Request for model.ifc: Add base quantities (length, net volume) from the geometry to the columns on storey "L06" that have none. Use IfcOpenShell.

First a look at what the model holds.

```python
import ifcopenshell
import ifcopenshell.util.element
import ifcopenshell.util.unit

model = ifcopenshell.open("model.ifc")
print(model.schema)
for unit_type in ("LENGTHUNIT", "AREAUNIT", "VOLUMEUNIT"):
    print(unit_type, ifcopenshell.util.unit.calculate_unit_scale(model, unit_type))
storey = next(s for s in model.by_type("IfcBuildingStorey") if s.Name == "L06")
columns = [e for e in ifcopenshell.util.element.get_decomposition(storey) if e.is_a("IfcColumn")]
for e in sorted(columns, key=lambda e: e.id()):
    print(e.id(), e.is_a(), e.Name, list(ifcopenshell.util.element.get_psets(e, qtos_only=True)), sep=" | ")
```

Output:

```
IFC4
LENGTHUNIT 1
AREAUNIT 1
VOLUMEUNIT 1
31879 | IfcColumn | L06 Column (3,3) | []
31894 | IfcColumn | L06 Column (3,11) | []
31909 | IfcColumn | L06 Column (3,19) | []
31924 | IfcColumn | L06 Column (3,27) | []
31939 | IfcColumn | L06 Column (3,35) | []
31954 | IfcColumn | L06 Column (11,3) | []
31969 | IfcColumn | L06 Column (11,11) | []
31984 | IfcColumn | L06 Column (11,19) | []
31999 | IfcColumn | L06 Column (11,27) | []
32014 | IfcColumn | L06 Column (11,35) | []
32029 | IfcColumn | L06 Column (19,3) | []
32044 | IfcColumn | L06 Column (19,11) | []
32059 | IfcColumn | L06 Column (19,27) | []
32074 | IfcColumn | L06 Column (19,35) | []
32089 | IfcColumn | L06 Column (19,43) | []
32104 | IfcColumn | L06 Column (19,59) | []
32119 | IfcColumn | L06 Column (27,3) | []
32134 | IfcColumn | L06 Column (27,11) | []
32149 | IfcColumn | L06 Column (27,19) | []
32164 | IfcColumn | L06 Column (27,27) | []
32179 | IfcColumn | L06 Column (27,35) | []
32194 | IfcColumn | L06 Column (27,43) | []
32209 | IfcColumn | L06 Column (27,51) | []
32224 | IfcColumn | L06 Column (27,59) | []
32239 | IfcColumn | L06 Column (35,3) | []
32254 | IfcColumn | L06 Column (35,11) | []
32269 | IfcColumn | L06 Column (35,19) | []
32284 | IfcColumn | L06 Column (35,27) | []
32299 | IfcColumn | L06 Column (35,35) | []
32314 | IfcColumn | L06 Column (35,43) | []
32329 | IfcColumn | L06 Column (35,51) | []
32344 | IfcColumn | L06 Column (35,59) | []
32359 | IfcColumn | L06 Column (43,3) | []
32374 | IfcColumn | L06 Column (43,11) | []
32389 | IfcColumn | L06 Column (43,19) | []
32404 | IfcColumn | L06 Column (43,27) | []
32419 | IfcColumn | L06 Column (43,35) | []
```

```python
import ifcopenshell
import ifcopenshell.api.pset
import ifcopenshell.geom
import ifcopenshell.util.element
import ifcopenshell.util.shape
import ifcopenshell.util.unit

model = ifcopenshell.open("model.ifc")
unit_scale = ifcopenshell.util.unit.calculate_unit_scale(model)
volume_scale = ifcopenshell.util.unit.calculate_unit_scale(model, "VOLUMEUNIT")
settings = ifcopenshell.geom.settings()

storey = next(s for s in model.by_type("IfcBuildingStorey") if s.Name == "L06")
columns = [e for e in ifcopenshell.util.element.get_decomposition(storey) if e.is_a("IfcColumn")]

for e in sorted(columns, key=lambda e: e.id()):
    if ifcopenshell.util.element.get_psets(e, qtos_only=True, should_inherit=False):
        continue
    # Geometry comes back in metres, in the element's own axes.
    shape = ifcopenshell.geom.create_shape(settings, e)
    values = {
        "Length": ifcopenshell.util.shape.get_z(shape.geometry) / unit_scale,
        "NetVolume": ifcopenshell.util.shape.get_volume(shape.geometry) / volume_scale,
    }
    qto = ifcopenshell.api.pset.add_qto(model, product=e, name="Qto_ColumnBaseQuantities")
    ifcopenshell.api.pset.edit_qto(model, qto=qto, properties=values)
    print(e.id(), {k: round(v, 3) for k, v in values.items()})

model.write("model_edited.ifc")
```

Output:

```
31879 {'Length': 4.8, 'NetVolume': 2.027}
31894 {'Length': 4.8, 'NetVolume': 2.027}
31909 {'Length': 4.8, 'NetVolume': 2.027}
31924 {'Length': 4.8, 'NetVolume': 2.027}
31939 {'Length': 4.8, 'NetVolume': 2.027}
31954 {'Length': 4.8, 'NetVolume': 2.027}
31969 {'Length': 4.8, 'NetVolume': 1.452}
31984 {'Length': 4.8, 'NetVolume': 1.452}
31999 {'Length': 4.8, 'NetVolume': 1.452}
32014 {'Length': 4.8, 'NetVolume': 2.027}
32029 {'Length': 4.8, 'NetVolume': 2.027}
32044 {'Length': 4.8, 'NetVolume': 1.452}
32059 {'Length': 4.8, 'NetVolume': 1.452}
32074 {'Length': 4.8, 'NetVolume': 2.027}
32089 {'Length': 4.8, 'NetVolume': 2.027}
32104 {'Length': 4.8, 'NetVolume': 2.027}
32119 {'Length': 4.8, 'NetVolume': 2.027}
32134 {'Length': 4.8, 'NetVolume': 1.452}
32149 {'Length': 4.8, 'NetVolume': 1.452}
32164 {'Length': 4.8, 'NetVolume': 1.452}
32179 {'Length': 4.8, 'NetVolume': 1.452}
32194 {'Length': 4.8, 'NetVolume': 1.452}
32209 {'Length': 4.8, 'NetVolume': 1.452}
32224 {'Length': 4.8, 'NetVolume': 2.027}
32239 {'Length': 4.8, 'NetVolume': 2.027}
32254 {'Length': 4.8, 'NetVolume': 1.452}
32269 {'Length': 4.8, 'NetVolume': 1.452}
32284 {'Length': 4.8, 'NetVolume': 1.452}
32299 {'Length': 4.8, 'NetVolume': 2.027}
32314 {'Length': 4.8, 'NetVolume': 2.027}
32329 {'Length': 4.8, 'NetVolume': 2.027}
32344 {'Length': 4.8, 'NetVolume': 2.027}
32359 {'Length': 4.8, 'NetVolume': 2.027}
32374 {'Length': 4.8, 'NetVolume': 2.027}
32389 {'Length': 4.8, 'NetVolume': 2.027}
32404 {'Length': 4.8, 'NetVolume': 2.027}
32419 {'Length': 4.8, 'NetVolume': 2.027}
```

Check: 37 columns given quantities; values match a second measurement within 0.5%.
